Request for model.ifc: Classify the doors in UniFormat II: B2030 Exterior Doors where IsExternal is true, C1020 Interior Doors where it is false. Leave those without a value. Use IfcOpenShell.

First a look at what the model holds.

```python
import ifcopenshell
import ifcopenshell.util.element

model = ifcopenshell.open("model.ifc")
print(model.schema)
print("classifications:", [c.Name for c in model.by_type("IfcClassification")])
values = [ifcopenshell.util.element.get_pset(e, "Pset_DoorCommon", "IsExternal") for e in model.by_type("IfcDoor")]
for value in (True, False, None):
    print("IsExternal", value, values.count(value))
```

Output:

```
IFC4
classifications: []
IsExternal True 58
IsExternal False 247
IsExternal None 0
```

```python
import ifcopenshell
import ifcopenshell.api.classification
import ifcopenshell.util.element

model = ifcopenshell.open("model.ifc")

system = ifcopenshell.api.classification.add_classification(model, classification="UniFormat II")

doors = model.by_type("IfcDoor")
external = {e: ifcopenshell.util.element.get_pset(e, "Pset_DoorCommon", "IsExternal") for e in doors}
for flag, code, name in ((True, "B2030", "Exterior Doors"), (False, "C1020", "Interior Doors")):
    products = [e for e in doors if external[e] is flag]
    ifcopenshell.api.classification.add_reference(
        model, products=products, classification=system, identification=code, name=name
    )
    print(code, len(products))

model.write("model_updated.ifc")
```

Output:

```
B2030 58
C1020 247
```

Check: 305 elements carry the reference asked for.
